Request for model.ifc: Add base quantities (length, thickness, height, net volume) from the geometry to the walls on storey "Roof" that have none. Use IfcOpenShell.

First a look at what the model holds.

```python
import ifcopenshell
import ifcopenshell.util.element
import ifcopenshell.util.unit

model = ifcopenshell.open("model.ifc")
print(model.schema)
for unit_type in ("LENGTHUNIT", "AREAUNIT", "VOLUMEUNIT"):
    print(unit_type, ifcopenshell.util.unit.calculate_unit_scale(model, unit_type))
storey = next(s for s in model.by_type("IfcBuildingStorey") if s.Name == "Roof")
walls = [e for e in ifcopenshell.util.element.get_decomposition(storey) if e.is_a("IfcWall")]
for e in sorted(walls, key=lambda e: e.id()):
    print(e.id(), e.is_a(), e.Name, list(ifcopenshell.util.element.get_psets(e, qtos_only=True)), sep=" | ")
```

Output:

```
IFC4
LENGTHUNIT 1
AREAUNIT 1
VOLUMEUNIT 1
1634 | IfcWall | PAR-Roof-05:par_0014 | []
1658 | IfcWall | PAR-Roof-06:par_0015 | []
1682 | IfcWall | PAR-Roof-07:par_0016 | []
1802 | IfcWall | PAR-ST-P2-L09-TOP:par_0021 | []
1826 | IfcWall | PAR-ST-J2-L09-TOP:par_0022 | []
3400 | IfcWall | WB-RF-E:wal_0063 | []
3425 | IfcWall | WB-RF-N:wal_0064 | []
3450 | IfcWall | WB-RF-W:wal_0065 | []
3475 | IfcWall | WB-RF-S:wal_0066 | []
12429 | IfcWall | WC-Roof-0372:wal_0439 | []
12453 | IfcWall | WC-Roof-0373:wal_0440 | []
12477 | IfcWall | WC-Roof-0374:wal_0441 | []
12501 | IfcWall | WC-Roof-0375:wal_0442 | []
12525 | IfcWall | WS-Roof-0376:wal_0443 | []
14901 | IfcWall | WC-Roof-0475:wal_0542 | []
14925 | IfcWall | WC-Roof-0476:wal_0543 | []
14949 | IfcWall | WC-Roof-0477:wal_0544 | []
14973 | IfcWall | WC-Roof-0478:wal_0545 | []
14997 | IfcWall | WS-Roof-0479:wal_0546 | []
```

```python
import ifcopenshell
import ifcopenshell.api.pset
import ifcopenshell.geom
import ifcopenshell.util.element
import ifcopenshell.util.shape
import ifcopenshell.util.unit

model = ifcopenshell.open("model.ifc")
unit_scale = ifcopenshell.util.unit.calculate_unit_scale(model)
volume_scale = ifcopenshell.util.unit.calculate_unit_scale(model, "VOLUMEUNIT")
settings = ifcopenshell.geom.settings()

storey = next(s for s in model.by_type("IfcBuildingStorey") if s.Name == "Roof")
walls = [e for e in ifcopenshell.util.element.get_decomposition(storey) if e.is_a("IfcWall")]

for e in sorted(walls, key=lambda e: e.id()):
    if ifcopenshell.util.element.get_psets(e, qtos_only=True, should_inherit=False):
        continue
    # Geometry comes back in metres, in the element's own axes.
    shape = ifcopenshell.geom.create_shape(settings, e)
    values = {
        "Length": ifcopenshell.util.shape.get_x(shape.geometry) / unit_scale,
        "Width": ifcopenshell.util.shape.get_y(shape.geometry) / unit_scale,
        "Height": ifcopenshell.util.shape.get_z(shape.geometry) / unit_scale,
        "NetVolume": ifcopenshell.util.shape.get_volume(shape.geometry) / volume_scale,
    }
    qto = ifcopenshell.api.pset.add_qto(model, product=e, name="Qto_WallBaseQuantities")
    ifcopenshell.api.pset.edit_qto(model, qto=qto, properties=values)
    print(e.id(), {k: round(v, 3) for k, v in values.items()})

model.write("model_rev.ifc")
```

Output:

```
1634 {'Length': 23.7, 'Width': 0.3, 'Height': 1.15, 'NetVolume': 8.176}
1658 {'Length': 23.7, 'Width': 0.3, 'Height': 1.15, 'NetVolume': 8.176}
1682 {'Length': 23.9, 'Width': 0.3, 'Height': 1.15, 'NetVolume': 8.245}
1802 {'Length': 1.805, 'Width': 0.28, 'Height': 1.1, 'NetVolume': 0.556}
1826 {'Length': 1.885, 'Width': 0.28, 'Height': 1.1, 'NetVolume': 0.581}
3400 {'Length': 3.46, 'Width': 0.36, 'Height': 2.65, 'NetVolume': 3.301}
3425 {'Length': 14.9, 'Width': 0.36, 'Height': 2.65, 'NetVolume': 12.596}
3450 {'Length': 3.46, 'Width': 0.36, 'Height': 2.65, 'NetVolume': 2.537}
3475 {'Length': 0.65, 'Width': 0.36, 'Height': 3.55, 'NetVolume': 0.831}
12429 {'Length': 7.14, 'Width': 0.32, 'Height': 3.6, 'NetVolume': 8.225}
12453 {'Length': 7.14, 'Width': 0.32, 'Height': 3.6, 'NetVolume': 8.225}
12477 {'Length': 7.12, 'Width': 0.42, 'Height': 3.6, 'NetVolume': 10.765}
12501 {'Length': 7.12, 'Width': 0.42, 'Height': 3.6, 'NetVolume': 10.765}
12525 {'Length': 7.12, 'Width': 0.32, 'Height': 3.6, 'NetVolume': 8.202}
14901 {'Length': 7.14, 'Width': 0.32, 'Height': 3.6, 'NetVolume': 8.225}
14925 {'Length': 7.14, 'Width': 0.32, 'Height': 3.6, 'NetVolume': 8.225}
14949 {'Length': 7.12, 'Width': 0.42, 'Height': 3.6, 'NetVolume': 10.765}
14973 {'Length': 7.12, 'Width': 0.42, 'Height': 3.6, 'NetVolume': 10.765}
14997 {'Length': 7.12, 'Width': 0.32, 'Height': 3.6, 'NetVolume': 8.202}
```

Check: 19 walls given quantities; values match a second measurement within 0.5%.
